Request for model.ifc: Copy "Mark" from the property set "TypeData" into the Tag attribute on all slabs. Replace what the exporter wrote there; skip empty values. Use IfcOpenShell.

First a look at what the model holds.

```python
import ifcopenshell
import ifcopenshell.util.element

model = ifcopenshell.open("model.ifc")
print(model.schema)
slabs = model.by_type("IfcSlab")
print(len(slabs), "slabs")
for e in slabs[:8]:
    source = ifcopenshell.util.element.get_pset(e, "TypeData", "Mark")
    target = e.Tag
    print(e.id(), repr(source), repr(target), sep=" | ")
```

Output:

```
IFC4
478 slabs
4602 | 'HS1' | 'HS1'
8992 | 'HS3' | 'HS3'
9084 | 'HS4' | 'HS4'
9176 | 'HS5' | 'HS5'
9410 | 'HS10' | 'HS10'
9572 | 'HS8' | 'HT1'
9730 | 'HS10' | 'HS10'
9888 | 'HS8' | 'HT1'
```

```python
import ifcopenshell
import ifcopenshell.util.element

model = ifcopenshell.open("model.ifc")

count = 0
for e in model.by_type("IfcSlab"):
    value = ifcopenshell.util.element.get_pset(e, "TypeData", "Mark")
    current = e.Tag
    if not value or not value.strip() or current == value:
        continue
    e.Tag = value
    count += 1

print(count, "slabs updated")

model.write("model_updated.ifc")
```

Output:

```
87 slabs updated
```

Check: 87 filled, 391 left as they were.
